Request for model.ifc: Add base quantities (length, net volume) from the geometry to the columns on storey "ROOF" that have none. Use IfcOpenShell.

First a look at what the model holds.

```python
import ifcopenshell
import ifcopenshell.util.element
import ifcopenshell.util.unit

model = ifcopenshell.open("model.ifc")
print(model.schema)
for unit_type in ("LENGTHUNIT", "AREAUNIT", "VOLUMEUNIT"):
    print(unit_type, ifcopenshell.util.unit.calculate_unit_scale(model, unit_type))
storey = next(s for s in model.by_type("IfcBuildingStorey") if s.Name == "ROOF")
columns = [e for e in ifcopenshell.util.element.get_decomposition(storey) if e.is_a("IfcColumn")]
for e in sorted(columns, key=lambda e: e.id()):
    print(e.id(), e.is_a(), e.Name, list(ifcopenshell.util.element.get_psets(e, qtos_only=True)), sep=" | ")
```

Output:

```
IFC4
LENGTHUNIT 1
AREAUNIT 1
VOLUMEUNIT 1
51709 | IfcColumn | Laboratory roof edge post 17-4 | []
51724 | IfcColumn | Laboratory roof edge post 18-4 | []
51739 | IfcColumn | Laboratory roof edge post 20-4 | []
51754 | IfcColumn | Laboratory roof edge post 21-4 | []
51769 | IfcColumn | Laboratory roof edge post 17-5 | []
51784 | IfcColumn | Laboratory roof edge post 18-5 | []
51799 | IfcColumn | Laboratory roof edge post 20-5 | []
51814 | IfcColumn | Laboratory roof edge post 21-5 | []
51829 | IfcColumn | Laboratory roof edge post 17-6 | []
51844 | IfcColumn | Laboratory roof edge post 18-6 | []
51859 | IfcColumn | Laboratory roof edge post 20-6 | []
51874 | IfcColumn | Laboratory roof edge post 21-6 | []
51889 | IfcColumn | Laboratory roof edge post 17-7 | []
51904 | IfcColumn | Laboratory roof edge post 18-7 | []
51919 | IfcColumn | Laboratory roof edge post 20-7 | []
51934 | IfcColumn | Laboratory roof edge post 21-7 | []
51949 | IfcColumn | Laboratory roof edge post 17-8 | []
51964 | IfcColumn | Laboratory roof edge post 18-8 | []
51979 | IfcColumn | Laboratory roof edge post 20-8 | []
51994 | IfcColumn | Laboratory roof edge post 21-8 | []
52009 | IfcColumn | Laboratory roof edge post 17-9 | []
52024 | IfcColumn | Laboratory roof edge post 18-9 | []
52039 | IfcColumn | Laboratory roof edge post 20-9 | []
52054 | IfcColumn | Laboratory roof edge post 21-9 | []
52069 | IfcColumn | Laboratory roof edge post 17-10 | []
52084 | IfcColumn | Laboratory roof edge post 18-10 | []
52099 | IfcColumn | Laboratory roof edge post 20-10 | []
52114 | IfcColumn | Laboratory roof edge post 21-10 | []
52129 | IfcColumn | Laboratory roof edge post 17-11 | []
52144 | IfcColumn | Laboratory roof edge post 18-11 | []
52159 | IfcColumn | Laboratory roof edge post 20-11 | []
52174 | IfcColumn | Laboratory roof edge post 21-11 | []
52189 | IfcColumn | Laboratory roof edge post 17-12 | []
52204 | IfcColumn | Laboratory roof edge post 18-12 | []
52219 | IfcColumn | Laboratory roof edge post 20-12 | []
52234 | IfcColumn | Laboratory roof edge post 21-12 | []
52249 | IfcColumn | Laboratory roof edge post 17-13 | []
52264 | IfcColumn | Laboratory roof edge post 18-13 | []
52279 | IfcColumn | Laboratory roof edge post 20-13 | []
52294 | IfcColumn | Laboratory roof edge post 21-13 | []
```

```python
import ifcopenshell
import ifcopenshell.api.pset
import ifcopenshell.geom
import ifcopenshell.util.element
import ifcopenshell.util.shape
import ifcopenshell.util.unit

model = ifcopenshell.open("model.ifc")
unit_scale = ifcopenshell.util.unit.calculate_unit_scale(model)
volume_scale = ifcopenshell.util.unit.calculate_unit_scale(model, "VOLUMEUNIT")
settings = ifcopenshell.geom.settings()

storey = next(s for s in model.by_type("IfcBuildingStorey") if s.Name == "ROOF")
columns = [e for e in ifcopenshell.util.element.get_decomposition(storey) if e.is_a("IfcColumn")]

for e in sorted(columns, key=lambda e: e.id()):
    if ifcopenshell.util.element.get_psets(e, qtos_only=True, should_inherit=False):
        continue
    # Geometry comes back in metres, in the element's own axes.
    shape = ifcopenshell.geom.create_shape(settings, e)
    values = {
        "Length": ifcopenshell.util.shape.get_z(shape.geometry) / unit_scale,
        "NetVolume": ifcopenshell.util.shape.get_volume(shape.geometry) / volume_scale,
    }
    qto = ifcopenshell.api.pset.add_qto(model, product=e, name="Qto_ColumnBaseQuantities")
    ifcopenshell.api.pset.edit_qto(model, qto=qto, properties=values)
    print(e.id(), {k: round(v, 3) for k, v in values.items()})

model.write("model_edited.ifc")
```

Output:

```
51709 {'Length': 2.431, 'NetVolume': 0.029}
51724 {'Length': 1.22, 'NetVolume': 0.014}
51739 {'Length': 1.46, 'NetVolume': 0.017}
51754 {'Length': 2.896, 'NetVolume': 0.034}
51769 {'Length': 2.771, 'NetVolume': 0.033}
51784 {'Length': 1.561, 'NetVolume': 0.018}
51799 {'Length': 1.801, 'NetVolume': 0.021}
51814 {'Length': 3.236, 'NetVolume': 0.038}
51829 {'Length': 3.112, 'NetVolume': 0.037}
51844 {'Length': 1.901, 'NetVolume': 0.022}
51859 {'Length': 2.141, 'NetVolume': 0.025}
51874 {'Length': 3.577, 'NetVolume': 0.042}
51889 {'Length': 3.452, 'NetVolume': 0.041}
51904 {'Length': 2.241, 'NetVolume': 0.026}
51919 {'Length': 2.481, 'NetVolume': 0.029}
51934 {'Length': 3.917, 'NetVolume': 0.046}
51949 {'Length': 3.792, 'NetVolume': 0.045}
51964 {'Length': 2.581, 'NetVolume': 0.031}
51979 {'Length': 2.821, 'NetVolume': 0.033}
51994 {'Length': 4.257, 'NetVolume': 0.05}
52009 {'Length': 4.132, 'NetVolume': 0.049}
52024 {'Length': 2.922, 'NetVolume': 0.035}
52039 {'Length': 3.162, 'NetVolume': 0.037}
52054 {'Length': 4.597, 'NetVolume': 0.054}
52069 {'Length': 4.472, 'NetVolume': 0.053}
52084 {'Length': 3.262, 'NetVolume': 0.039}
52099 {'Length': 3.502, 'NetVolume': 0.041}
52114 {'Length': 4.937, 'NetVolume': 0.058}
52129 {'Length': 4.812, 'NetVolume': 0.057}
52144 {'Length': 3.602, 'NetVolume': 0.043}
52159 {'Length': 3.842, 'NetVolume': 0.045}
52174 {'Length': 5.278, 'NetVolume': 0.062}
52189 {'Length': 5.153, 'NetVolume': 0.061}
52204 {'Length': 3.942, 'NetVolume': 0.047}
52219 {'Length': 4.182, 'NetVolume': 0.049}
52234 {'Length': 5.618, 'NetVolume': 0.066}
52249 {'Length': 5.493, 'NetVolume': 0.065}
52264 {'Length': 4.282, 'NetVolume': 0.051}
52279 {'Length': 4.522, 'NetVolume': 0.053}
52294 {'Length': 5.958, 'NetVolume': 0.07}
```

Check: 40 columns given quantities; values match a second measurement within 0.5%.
